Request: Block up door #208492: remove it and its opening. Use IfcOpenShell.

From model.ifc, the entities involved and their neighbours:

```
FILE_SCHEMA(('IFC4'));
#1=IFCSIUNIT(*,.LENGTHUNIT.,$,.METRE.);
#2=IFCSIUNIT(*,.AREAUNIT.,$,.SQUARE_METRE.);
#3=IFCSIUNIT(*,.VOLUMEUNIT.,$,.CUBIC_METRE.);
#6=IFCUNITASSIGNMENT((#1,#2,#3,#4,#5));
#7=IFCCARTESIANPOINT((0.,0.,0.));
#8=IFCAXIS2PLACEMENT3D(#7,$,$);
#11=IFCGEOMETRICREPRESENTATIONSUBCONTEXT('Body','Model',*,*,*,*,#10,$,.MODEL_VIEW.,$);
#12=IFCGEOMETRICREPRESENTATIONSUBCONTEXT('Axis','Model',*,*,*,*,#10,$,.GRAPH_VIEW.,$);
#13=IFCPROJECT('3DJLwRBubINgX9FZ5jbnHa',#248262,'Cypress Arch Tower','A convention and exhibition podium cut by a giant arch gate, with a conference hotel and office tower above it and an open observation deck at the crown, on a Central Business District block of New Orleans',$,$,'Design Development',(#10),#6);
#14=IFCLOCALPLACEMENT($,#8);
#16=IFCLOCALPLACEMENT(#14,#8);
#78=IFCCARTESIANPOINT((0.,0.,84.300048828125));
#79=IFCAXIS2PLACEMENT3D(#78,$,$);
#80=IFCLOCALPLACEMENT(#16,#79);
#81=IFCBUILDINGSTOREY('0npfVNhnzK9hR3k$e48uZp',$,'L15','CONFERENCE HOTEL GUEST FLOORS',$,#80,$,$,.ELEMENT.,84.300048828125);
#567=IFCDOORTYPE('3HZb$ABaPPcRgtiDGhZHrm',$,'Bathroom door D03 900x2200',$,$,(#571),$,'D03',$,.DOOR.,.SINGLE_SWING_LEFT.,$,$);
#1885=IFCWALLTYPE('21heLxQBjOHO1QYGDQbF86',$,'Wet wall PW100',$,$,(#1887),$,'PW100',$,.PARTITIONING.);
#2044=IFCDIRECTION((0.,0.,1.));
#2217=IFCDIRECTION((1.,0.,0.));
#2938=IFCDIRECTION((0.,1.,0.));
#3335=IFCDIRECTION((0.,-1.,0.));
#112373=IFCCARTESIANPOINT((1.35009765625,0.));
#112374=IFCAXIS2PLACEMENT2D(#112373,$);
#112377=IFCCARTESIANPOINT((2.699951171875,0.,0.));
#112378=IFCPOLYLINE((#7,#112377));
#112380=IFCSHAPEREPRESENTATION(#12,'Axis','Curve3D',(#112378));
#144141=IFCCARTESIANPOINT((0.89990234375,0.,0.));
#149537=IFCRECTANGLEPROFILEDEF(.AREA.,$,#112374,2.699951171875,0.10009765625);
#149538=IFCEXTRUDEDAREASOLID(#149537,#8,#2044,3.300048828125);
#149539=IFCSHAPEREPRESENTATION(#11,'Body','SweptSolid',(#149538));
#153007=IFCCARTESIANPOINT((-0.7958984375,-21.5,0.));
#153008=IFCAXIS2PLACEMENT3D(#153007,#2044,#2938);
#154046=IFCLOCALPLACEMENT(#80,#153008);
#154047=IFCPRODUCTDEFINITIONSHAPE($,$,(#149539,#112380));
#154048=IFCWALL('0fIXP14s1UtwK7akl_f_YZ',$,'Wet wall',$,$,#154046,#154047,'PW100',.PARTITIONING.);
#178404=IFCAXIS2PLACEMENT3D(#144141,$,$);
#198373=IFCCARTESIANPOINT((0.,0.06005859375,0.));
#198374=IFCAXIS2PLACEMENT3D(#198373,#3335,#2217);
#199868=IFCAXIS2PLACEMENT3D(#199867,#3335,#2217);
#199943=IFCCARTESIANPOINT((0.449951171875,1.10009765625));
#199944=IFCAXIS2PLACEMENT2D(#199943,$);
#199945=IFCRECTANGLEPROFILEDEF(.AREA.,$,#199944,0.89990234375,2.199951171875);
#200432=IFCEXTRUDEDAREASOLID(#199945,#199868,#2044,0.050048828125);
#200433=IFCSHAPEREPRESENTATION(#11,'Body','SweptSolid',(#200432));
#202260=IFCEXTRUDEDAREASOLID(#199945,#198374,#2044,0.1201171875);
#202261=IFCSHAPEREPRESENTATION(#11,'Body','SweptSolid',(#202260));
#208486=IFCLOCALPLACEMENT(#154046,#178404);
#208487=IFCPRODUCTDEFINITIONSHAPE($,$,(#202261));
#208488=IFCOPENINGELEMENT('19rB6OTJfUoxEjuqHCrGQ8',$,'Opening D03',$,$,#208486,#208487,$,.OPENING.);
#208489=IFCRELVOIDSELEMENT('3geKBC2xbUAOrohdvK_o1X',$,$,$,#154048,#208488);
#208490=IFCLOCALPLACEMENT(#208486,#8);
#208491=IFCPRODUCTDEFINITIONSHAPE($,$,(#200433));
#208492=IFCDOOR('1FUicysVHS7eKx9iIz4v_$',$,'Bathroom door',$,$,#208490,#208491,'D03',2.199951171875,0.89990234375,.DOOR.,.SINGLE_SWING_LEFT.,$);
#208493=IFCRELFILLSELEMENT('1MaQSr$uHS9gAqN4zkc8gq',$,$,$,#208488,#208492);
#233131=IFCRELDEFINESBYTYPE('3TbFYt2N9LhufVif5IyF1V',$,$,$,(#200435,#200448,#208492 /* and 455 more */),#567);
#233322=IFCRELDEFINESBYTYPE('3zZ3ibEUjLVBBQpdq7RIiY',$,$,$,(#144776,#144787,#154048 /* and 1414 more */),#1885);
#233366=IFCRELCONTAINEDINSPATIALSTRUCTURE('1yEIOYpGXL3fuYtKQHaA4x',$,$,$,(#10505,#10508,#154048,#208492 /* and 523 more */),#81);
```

```python
import ifcopenshell
import ifcopenshell.api.feature
import ifcopenshell.api.root
import ifcopenshell.geom
import ifcopenshell.util.shape

model = ifcopenshell.open("model.ifc")
settings = ifcopenshell.geom.settings()


def volume(element):
    """Net volume in cubic metres, openings subtracted."""
    shape = ifcopenshell.geom.create_shape(settings, element)
    return ifcopenshell.util.shape.get_volume(shape.geometry)


door = model.by_id(208492)
opening = door.FillsVoids[0].RelatingOpeningElement
wall = opening.VoidsElements[0].RelatingBuildingElement
before = volume(wall)

ifcopenshell.api.root.remove_product(model, product=door)
ifcopenshell.api.feature.remove_feature(model, feature=opening)

after = volume(wall)

print(f"wall volume {before:.3f} -> {after:.3f} m3")

model.write("model_updated.ifc")
```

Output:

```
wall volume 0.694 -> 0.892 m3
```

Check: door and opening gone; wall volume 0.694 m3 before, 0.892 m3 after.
